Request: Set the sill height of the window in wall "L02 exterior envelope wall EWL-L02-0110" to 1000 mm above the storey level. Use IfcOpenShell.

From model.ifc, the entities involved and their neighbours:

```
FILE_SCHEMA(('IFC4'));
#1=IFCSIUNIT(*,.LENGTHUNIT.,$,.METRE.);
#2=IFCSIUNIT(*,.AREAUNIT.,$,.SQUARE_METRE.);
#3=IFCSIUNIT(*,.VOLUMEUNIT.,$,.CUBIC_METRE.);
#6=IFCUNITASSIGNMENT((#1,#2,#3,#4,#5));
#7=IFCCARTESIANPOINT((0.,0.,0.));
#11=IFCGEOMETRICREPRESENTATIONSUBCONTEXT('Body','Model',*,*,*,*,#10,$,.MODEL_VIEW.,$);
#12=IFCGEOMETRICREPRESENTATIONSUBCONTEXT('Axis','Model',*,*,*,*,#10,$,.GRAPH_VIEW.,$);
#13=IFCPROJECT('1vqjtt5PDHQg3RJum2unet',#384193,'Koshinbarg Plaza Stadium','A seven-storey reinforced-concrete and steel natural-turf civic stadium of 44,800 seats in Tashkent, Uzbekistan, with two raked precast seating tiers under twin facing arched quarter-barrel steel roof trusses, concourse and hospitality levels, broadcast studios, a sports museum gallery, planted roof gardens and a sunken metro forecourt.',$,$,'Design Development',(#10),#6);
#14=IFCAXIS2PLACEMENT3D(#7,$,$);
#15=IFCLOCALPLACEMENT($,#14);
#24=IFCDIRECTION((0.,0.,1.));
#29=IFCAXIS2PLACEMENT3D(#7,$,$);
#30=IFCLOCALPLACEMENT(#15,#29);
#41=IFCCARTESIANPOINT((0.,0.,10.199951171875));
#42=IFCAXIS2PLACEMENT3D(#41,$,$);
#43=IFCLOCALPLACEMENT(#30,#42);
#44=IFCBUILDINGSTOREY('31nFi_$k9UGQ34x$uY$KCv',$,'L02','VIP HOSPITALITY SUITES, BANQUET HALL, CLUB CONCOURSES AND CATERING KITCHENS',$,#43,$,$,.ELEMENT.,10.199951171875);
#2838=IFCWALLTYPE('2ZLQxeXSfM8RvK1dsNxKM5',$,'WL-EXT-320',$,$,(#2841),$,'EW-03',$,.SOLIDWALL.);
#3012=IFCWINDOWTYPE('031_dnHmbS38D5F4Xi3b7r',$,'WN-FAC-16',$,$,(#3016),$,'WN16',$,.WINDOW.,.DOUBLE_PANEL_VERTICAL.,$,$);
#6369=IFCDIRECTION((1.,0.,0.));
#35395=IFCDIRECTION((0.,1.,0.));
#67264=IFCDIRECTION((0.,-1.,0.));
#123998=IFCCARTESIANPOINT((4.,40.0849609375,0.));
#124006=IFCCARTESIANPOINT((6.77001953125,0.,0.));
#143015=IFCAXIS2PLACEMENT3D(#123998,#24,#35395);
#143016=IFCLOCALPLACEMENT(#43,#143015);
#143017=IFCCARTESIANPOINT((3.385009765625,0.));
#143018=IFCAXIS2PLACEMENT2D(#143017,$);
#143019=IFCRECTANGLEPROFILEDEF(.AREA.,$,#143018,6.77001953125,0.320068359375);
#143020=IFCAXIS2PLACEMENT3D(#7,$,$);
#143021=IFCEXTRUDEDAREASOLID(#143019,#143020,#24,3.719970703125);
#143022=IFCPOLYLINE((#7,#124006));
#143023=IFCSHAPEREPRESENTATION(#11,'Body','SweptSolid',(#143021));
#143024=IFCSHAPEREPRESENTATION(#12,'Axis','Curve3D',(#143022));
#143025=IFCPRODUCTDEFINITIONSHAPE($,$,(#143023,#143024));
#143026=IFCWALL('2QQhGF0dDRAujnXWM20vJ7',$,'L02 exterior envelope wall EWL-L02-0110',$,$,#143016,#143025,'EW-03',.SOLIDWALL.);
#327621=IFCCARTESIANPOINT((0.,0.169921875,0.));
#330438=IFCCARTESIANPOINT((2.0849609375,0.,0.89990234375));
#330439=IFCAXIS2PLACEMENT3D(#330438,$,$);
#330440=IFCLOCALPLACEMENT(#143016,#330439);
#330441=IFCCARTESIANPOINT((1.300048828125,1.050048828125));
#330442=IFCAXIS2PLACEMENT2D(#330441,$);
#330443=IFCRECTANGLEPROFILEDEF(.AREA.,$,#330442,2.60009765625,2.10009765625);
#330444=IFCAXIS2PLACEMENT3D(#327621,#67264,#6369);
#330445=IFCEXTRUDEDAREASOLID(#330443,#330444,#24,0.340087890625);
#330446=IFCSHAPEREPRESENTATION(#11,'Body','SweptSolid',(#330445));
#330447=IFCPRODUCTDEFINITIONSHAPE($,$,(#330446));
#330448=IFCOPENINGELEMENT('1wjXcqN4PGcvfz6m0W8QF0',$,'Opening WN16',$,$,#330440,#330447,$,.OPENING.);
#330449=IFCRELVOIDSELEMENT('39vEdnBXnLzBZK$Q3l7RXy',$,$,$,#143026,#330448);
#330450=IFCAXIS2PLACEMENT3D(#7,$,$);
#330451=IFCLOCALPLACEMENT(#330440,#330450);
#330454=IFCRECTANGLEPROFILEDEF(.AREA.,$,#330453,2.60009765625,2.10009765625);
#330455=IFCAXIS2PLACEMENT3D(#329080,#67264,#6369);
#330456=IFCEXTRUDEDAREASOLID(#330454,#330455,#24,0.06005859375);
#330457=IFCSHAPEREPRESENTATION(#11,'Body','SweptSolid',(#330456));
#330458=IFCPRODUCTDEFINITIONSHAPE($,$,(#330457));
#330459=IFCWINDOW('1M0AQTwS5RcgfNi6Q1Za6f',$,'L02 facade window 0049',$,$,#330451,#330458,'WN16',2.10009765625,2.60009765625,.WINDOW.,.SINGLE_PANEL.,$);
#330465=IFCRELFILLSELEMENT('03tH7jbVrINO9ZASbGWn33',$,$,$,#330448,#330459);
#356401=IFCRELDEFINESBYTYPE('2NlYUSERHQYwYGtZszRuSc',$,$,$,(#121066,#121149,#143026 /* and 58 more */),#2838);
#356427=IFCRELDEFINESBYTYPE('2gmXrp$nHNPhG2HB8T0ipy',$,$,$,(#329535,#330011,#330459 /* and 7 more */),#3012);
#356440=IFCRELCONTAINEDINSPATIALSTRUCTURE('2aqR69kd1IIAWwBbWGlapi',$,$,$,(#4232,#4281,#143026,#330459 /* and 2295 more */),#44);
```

```python
import numpy as np
import ifcopenshell
import ifcopenshell.api.geometry
import ifcopenshell.geom
import ifcopenshell.util.element
import ifcopenshell.util.placement
import ifcopenshell.util.shape
import ifcopenshell.util.unit

model = ifcopenshell.open("model.ifc")
unit_scale = ifcopenshell.util.unit.calculate_unit_scale(model)

window = model.by_guid("1M0AQTwS5RcgfNi6Q1Za6f")
opening = window.FillsVoids[0].RelatingOpeningElement
storey = ifcopenshell.util.element.get_container(window, ifc_class="IfcBuildingStorey")
level = ifcopenshell.util.placement.get_local_placement(storey.ObjectPlacement)[2, 3]

# The opening's origin need not be at the sill, so measure its lowest point.
shape = ifcopenshell.geom.create_shape(ifcopenshell.geom.settings(), opening)
bottom = ifcopenshell.util.shape.get_shape_bottom_elevation(shape, shape.geometry) / unit_scale
dz = level + 1 / unit_scale - bottom

shift = np.array([0.0, 0.0, dz])
# The window is placed relative to its opening, so it follows when the opening moves.
matrix = ifcopenshell.util.placement.get_local_placement(opening.ObjectPlacement)
matrix[:3, 3] += shift
ifcopenshell.api.geometry.edit_object_placement(
    model, product=opening, matrix=matrix, is_si=False, should_transform_children=True
)

print(f"moved by {dz * unit_scale:+.3f} m")

model.write("model_v2.ifc")
```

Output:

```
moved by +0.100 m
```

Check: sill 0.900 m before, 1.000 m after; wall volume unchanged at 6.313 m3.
